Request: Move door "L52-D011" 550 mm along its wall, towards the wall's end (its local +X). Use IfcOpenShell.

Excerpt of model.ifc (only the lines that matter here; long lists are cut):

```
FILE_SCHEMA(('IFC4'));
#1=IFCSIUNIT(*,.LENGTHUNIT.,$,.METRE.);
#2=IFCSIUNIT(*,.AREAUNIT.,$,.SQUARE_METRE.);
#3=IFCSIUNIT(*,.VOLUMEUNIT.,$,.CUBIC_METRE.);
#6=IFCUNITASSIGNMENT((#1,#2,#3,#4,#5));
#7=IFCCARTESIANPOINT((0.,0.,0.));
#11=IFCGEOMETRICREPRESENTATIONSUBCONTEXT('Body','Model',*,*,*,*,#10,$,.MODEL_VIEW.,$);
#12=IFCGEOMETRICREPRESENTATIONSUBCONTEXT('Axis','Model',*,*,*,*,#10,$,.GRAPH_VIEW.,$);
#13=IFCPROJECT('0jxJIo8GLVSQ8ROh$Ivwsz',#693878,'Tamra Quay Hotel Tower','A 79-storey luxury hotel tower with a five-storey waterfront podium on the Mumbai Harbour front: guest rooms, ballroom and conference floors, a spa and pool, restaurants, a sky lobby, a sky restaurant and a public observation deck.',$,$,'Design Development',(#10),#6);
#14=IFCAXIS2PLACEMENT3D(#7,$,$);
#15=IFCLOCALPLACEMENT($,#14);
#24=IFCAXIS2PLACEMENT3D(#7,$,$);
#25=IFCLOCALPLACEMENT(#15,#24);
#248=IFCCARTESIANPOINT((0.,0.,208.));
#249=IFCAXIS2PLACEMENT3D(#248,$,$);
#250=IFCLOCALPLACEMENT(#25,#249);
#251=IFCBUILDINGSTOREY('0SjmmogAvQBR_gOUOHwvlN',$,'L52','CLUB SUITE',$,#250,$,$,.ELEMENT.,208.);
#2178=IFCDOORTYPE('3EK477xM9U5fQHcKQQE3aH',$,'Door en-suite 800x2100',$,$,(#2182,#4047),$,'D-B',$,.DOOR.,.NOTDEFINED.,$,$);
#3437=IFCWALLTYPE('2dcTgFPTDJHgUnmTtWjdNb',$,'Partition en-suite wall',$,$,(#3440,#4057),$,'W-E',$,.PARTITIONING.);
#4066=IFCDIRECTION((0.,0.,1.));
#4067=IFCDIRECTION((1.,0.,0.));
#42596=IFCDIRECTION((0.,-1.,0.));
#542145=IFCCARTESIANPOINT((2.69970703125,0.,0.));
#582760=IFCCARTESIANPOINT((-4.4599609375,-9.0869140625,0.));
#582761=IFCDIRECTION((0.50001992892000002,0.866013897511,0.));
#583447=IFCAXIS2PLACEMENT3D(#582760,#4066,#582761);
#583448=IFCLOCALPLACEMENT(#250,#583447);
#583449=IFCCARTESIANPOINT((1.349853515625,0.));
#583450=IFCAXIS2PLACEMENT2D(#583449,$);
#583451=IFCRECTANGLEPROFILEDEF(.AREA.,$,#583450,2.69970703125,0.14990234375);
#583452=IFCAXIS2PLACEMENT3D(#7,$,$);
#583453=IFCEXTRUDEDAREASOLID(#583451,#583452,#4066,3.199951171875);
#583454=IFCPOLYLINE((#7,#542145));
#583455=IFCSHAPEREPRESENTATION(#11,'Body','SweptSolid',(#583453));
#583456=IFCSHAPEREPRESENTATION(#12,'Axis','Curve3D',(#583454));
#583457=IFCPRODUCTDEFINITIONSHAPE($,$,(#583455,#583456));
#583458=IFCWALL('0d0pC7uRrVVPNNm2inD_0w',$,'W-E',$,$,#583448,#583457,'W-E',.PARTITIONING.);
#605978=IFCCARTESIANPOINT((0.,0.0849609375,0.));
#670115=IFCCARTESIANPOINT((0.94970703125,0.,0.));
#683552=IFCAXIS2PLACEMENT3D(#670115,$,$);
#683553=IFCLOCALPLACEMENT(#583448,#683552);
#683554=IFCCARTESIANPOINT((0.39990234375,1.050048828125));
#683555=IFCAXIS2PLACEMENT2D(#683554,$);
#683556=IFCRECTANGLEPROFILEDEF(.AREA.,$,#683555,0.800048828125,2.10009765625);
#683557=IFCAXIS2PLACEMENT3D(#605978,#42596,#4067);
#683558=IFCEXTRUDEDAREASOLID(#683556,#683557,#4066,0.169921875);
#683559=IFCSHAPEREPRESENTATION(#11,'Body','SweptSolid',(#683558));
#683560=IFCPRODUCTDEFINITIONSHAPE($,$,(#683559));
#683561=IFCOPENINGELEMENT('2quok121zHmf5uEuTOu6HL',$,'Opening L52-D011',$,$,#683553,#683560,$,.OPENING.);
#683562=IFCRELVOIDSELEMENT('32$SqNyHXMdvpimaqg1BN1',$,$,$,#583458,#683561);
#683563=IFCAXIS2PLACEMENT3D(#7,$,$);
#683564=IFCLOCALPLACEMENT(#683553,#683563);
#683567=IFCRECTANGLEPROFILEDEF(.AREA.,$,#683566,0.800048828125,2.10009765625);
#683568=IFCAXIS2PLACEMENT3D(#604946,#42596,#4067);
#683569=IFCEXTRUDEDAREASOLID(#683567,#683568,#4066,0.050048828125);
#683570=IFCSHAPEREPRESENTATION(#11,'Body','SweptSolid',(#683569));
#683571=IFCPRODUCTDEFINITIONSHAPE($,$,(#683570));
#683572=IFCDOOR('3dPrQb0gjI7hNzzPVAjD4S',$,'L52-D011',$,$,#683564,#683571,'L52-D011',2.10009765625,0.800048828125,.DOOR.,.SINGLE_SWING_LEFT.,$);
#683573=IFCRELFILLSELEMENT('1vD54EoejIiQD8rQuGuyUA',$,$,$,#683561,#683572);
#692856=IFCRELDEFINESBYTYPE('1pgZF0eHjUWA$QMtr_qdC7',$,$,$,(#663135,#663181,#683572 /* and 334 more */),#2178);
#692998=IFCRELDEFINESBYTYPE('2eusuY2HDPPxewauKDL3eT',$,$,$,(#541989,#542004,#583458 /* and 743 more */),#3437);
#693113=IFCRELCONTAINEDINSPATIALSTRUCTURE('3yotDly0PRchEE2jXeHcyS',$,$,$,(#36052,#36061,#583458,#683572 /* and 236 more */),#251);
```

```python
import ifcopenshell
import ifcopenshell.api.geometry
import ifcopenshell.util.placement

model = ifcopenshell.open("model.ifc")

door = model.by_id(683572)
opening = door.FillsVoids[0].RelatingOpeningElement
wall = opening.VoidsElements[0].RelatingBuildingElement

wall_matrix = ifcopenshell.util.placement.get_local_placement(wall.ObjectPlacement)
shift = wall_matrix[:3, 0] * 0.55
before = ifcopenshell.util.placement.get_local_placement(door.ObjectPlacement)[:3, 3].copy()

# The door is placed relative to its opening, so it follows when the opening moves.
matrix = ifcopenshell.util.placement.get_local_placement(opening.ObjectPlacement)
matrix[:3, 3] += shift
ifcopenshell.api.geometry.edit_object_placement(
    model, product=opening, matrix=matrix, is_si=False, should_transform_children=True
)

after = ifcopenshell.util.placement.get_local_placement(door.ObjectPlacement)[:3, 3]
print("door moved by", (after - before).round(3) + 0.0)

model.write("model_edited.ifc")
```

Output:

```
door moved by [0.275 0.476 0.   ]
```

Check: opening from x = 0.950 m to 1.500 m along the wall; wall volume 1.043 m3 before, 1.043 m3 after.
